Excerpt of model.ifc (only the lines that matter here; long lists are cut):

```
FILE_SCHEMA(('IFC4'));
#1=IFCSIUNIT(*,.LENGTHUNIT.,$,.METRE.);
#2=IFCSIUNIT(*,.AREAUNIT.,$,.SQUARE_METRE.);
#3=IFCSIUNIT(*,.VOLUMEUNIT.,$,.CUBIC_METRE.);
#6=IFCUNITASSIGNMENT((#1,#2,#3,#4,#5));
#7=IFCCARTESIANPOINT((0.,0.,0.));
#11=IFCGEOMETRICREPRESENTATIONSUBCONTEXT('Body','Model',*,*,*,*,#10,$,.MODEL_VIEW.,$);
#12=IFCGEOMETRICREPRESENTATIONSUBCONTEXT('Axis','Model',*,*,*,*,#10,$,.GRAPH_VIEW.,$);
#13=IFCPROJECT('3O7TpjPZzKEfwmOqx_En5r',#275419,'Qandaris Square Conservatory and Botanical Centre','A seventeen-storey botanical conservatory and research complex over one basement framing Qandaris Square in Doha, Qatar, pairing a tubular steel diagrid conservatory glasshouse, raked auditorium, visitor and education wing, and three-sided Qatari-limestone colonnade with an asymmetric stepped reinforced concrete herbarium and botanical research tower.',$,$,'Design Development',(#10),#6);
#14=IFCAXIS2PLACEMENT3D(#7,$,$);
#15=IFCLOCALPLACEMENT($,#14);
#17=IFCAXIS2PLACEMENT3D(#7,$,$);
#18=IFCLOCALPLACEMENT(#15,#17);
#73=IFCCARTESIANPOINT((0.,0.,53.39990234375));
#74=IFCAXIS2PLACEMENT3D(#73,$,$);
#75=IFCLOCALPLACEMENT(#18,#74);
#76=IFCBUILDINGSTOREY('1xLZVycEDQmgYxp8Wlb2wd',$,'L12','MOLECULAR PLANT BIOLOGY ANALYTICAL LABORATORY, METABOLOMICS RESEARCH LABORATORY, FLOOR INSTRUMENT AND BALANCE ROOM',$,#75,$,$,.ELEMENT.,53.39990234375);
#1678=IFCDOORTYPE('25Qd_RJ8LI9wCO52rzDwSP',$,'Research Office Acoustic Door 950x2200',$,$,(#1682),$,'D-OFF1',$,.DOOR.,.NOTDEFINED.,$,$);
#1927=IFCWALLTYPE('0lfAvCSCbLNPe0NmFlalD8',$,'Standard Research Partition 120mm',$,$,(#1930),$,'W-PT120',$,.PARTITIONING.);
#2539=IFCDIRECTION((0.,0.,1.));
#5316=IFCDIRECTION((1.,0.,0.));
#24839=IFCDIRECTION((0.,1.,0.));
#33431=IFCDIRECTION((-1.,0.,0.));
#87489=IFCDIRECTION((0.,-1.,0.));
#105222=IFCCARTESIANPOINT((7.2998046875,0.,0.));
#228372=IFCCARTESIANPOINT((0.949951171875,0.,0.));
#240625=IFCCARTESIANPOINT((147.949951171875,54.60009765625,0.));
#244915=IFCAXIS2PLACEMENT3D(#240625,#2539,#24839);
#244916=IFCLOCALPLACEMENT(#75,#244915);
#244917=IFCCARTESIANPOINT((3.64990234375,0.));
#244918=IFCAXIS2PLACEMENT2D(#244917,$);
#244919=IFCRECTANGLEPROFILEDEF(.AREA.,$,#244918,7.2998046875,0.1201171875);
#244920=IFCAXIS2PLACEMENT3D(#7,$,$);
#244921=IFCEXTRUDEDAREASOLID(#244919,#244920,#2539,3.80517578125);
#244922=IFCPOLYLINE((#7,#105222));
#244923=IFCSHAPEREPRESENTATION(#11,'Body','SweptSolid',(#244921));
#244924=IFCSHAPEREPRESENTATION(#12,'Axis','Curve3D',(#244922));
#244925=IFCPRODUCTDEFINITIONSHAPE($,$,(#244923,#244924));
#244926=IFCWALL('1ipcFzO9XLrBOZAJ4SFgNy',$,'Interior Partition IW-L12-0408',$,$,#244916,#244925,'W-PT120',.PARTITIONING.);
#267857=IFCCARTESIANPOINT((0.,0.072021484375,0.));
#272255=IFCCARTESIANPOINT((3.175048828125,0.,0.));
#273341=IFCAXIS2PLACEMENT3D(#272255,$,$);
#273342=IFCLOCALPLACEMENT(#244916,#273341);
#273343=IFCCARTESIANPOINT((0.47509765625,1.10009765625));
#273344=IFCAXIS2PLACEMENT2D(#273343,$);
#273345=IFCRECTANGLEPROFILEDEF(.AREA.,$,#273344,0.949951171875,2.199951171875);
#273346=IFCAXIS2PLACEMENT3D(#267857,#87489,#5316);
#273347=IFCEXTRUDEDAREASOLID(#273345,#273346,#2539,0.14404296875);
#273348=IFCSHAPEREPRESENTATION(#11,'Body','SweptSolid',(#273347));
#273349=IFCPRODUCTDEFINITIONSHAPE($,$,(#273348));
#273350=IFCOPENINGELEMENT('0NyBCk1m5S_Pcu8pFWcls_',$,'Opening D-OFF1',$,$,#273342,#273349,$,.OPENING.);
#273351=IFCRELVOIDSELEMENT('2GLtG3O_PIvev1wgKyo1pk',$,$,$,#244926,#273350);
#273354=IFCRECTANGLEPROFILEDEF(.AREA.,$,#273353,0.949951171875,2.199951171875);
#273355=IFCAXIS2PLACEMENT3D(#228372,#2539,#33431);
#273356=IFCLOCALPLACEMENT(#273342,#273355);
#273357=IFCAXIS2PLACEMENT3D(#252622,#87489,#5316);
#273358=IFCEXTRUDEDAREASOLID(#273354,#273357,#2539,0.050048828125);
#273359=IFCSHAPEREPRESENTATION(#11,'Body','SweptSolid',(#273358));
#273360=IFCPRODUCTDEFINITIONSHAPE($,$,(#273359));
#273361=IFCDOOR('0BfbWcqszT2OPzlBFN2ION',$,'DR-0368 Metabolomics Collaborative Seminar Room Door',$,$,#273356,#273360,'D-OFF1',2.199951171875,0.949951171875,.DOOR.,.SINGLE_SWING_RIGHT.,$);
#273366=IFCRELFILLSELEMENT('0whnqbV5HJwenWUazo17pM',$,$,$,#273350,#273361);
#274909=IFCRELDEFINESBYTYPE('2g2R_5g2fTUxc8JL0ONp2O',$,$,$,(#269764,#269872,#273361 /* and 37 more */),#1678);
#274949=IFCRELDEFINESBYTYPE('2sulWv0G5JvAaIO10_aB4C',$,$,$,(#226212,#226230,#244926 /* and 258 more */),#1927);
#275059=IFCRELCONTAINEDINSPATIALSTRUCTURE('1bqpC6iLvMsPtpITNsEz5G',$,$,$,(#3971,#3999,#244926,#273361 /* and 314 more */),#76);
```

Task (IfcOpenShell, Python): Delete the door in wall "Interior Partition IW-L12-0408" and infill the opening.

```python
import ifcopenshell
import ifcopenshell.api.feature
import ifcopenshell.api.root
import ifcopenshell.geom
import ifcopenshell.util.shape

model = ifcopenshell.open("model.ifc")
settings = ifcopenshell.geom.settings()


def volume(element):
    """Net volume in cubic metres, openings subtracted."""
    shape = ifcopenshell.geom.create_shape(settings, element)
    return ifcopenshell.util.shape.get_volume(shape.geometry)


door = model.by_id(273361)
opening = door.FillsVoids[0].RelatingOpeningElement
wall = opening.VoidsElements[0].RelatingBuildingElement
before = volume(wall)

ifcopenshell.api.root.remove_product(model, product=door)
ifcopenshell.api.feature.remove_feature(model, feature=opening)

after = volume(wall)

print(f"wall volume {before:.3f} -> {after:.3f} m3")

model.write("model_rev.ifc")
```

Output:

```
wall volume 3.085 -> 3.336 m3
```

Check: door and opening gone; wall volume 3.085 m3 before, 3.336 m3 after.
